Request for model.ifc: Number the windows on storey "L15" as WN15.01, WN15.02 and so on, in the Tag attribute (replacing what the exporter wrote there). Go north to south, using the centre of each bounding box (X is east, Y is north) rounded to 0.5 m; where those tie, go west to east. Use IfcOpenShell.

First a look at what the model holds.

```python
import ifcopenshell
import ifcopenshell.util.element
import ifcopenshell.util.placement

model = ifcopenshell.open("model.ifc")
print(model.schema)
storey = next(s for s in model.by_type("IfcBuildingStorey") if s.Name == "L15")
windows = [e for e in ifcopenshell.util.element.get_decomposition(storey) if e.is_a("IfcWindow")]
for e in sorted(windows, key=lambda e: e.id()):
    origin = ifcopenshell.util.placement.get_local_placement(e.ObjectPlacement)[:3, 3]
    print(e.id(), e.Tag, e.Name, origin.round(2) + 0.0, sep=" | ")
```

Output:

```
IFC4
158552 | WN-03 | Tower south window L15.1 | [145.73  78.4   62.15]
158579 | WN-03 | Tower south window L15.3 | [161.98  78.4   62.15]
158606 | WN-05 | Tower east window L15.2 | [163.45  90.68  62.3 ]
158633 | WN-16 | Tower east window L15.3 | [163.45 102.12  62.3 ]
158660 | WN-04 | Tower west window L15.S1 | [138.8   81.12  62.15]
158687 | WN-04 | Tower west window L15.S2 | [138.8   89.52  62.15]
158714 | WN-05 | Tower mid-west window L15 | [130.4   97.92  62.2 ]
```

```python
import ifcopenshell
import ifcopenshell.geom
import ifcopenshell.util.element
import ifcopenshell.util.shape

model = ifcopenshell.open("model.ifc")
settings = ifcopenshell.geom.settings()
settings.set("use-world-coords", True)


def centre(element):
    shape = ifcopenshell.geom.create_shape(settings, element)
    return ifcopenshell.util.shape.get_bbox_centroid(shape.geometry)


storey = next(s for s in model.by_type("IfcBuildingStorey") if s.Name == "L15")
windows = [e for e in ifcopenshell.util.element.get_decomposition(storey) if e.is_a("IfcWindow")]

# Insertion points can sit at a corner or the storey origin, so sort by the geometry (in metres).
centres = {e: centre(e) for e in windows}
windows.sort(key=lambda e: (-round(centres[e][1] / 0.5), centres[e][0]))

for i, e in enumerate(windows, start=1):
    number = f"WN15.{i:02d}"
    e.Tag = number
    print(e.id(), number)

model.write("model_v2.ifc")
```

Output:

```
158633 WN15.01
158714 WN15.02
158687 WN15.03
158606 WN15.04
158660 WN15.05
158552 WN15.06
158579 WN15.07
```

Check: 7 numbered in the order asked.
